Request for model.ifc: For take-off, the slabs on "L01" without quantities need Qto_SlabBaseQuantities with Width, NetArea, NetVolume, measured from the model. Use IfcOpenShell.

First a look at what the model holds.

```python
import ifcopenshell
import ifcopenshell.util.element
import ifcopenshell.util.unit

model = ifcopenshell.open("model.ifc")
print(model.schema)
for unit_type in ("LENGTHUNIT", "AREAUNIT", "VOLUMEUNIT"):
    print(unit_type, ifcopenshell.util.unit.calculate_unit_scale(model, unit_type))
storey = next(s for s in model.by_type("IfcBuildingStorey") if s.Name == "L01")
slabs = [e for e in ifcopenshell.util.element.get_decomposition(storey) if e.is_a("IfcSlab")]
for e in sorted(slabs, key=lambda e: e.id()):
    print(e.id(), e.is_a(), e.Name, list(ifcopenshell.util.element.get_psets(e, qtos_only=True)), sep=" | ")
```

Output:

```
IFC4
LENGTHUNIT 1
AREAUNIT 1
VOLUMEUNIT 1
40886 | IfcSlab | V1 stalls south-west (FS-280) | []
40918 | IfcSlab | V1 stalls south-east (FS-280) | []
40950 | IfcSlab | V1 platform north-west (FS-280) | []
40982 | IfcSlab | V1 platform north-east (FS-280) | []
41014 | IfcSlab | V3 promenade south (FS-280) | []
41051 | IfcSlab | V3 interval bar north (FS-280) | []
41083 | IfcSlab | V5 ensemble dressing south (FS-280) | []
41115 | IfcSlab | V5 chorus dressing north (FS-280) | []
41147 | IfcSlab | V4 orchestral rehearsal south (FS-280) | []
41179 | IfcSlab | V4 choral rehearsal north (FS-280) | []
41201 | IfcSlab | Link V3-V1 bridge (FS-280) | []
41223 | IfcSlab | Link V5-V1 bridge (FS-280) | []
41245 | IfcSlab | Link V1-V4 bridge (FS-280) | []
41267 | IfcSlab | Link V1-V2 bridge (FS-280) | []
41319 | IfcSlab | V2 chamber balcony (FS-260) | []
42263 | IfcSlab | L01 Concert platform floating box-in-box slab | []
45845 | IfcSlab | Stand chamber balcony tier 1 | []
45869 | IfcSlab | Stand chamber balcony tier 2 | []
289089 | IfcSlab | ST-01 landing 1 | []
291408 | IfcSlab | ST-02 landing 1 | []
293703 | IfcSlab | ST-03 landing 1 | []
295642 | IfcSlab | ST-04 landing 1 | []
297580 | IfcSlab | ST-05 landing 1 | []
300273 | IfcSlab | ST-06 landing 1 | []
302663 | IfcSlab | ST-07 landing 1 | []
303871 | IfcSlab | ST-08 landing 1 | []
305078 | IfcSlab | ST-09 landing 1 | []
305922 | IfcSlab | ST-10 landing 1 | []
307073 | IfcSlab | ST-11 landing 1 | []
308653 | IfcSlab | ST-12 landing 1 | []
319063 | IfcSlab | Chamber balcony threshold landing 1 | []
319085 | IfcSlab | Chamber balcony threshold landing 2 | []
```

```python
import ifcopenshell
import ifcopenshell.api.pset
import ifcopenshell.geom
import ifcopenshell.util.element
import ifcopenshell.util.shape
import ifcopenshell.util.unit

model = ifcopenshell.open("model.ifc")
unit_scale = ifcopenshell.util.unit.calculate_unit_scale(model)
area_scale = ifcopenshell.util.unit.calculate_unit_scale(model, "AREAUNIT")
volume_scale = ifcopenshell.util.unit.calculate_unit_scale(model, "VOLUMEUNIT")
settings = ifcopenshell.geom.settings()

storey = next(s for s in model.by_type("IfcBuildingStorey") if s.Name == "L01")
slabs = [e for e in ifcopenshell.util.element.get_decomposition(storey) if e.is_a("IfcSlab")]

for e in sorted(slabs, key=lambda e: e.id()):
    if ifcopenshell.util.element.get_psets(e, qtos_only=True, should_inherit=False):
        continue
    # Geometry comes back in metres, in the element's own axes.
    shape = ifcopenshell.geom.create_shape(settings, e)
    values = {
        "Width": ifcopenshell.util.shape.get_z(shape.geometry) / unit_scale,
        "NetArea": ifcopenshell.util.shape.get_footprint_area(shape.geometry) / area_scale,
        "NetVolume": ifcopenshell.util.shape.get_volume(shape.geometry) / volume_scale,
    }
    qto = ifcopenshell.api.pset.add_qto(model, product=e, name="Qto_SlabBaseQuantities")
    ifcopenshell.api.pset.edit_qto(model, qto=qto, properties=values)
    print(e.id(), {k: round(v, 3) for k, v in values.items()})

model.write("model-out.ifc")
```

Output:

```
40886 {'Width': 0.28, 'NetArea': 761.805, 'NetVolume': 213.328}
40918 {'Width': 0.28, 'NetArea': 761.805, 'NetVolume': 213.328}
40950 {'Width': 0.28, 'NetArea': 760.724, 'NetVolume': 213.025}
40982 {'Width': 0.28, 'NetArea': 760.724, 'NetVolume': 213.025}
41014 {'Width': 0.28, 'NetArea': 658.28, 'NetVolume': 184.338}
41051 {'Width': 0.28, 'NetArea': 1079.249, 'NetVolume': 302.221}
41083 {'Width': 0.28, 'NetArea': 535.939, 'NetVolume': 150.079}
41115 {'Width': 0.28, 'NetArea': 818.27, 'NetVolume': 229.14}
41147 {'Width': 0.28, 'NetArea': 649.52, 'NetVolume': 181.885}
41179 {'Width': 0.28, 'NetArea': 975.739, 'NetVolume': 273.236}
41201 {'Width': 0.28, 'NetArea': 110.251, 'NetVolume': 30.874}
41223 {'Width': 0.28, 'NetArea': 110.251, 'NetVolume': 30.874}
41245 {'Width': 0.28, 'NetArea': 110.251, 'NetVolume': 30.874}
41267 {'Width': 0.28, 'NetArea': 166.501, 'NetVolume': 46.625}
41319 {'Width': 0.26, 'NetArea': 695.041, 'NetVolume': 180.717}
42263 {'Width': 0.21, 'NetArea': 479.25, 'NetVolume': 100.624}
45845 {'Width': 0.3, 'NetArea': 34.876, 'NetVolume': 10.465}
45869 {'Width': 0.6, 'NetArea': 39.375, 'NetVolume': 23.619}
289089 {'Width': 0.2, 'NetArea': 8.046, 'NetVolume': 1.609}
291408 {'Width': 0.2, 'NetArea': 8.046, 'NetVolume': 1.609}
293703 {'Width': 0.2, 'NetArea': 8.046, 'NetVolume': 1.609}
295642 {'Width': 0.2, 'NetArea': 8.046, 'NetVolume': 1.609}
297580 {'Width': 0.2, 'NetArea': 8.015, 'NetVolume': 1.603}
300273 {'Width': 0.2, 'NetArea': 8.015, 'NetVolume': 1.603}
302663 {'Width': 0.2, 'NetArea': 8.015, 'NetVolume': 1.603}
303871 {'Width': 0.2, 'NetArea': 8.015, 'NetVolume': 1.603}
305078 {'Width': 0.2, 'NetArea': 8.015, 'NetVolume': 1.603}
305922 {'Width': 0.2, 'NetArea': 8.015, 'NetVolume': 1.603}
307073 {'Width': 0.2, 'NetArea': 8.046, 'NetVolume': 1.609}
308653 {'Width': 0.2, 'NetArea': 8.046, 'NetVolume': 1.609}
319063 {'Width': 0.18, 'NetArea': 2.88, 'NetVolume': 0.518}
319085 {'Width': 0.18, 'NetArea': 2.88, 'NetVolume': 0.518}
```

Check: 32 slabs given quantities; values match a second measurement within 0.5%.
